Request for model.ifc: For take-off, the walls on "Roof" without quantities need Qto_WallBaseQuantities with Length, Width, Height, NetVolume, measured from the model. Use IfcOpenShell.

First a look at what the model holds.

```python
import ifcopenshell
import ifcopenshell.util.element
import ifcopenshell.util.unit

model = ifcopenshell.open("model.ifc")
print(model.schema)
for unit_type in ("LENGTHUNIT", "AREAUNIT", "VOLUMEUNIT"):
    print(unit_type, ifcopenshell.util.unit.calculate_unit_scale(model, unit_type))
storey = next(s for s in model.by_type("IfcBuildingStorey") if s.Name == "Roof")
walls = [e for e in ifcopenshell.util.element.get_decomposition(storey) if e.is_a("IfcWall")]
for e in sorted(walls, key=lambda e: e.id()):
    print(e.id(), e.is_a(), e.Name, list(ifcopenshell.util.element.get_psets(e, qtos_only=True)), sep=" | ")
```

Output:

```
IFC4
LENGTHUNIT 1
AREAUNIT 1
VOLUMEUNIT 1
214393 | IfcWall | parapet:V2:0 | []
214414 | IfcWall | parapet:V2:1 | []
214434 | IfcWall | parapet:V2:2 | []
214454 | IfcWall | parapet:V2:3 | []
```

```python
import ifcopenshell
import ifcopenshell.api.pset
import ifcopenshell.geom
import ifcopenshell.util.element
import ifcopenshell.util.shape
import ifcopenshell.util.unit

model = ifcopenshell.open("model.ifc")
unit_scale = ifcopenshell.util.unit.calculate_unit_scale(model)
volume_scale = ifcopenshell.util.unit.calculate_unit_scale(model, "VOLUMEUNIT")
settings = ifcopenshell.geom.settings()

storey = next(s for s in model.by_type("IfcBuildingStorey") if s.Name == "Roof")
walls = [e for e in ifcopenshell.util.element.get_decomposition(storey) if e.is_a("IfcWall")]

for e in sorted(walls, key=lambda e: e.id()):
    if ifcopenshell.util.element.get_psets(e, qtos_only=True, should_inherit=False):
        continue
    # Geometry comes back in metres, in the element's own axes.
    shape = ifcopenshell.geom.create_shape(settings, e)
    values = {
        "Length": ifcopenshell.util.shape.get_x(shape.geometry) / unit_scale,
        "Width": ifcopenshell.util.shape.get_y(shape.geometry) / unit_scale,
        "Height": ifcopenshell.util.shape.get_z(shape.geometry) / unit_scale,
        "NetVolume": ifcopenshell.util.shape.get_volume(shape.geometry) / volume_scale,
    }
    qto = ifcopenshell.api.pset.add_qto(model, product=e, name="Qto_WallBaseQuantities")
    ifcopenshell.api.pset.edit_qto(model, qto=qto, properties=values)
    print(e.id(), {k: round(v, 3) for k, v in values.items()})

model.write("model_updated.ifc")
```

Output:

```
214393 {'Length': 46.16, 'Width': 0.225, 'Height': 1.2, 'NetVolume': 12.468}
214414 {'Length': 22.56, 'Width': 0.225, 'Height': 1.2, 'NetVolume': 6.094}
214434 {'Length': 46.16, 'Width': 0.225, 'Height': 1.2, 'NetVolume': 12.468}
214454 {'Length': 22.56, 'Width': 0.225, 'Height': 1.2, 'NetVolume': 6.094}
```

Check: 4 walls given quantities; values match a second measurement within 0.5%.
